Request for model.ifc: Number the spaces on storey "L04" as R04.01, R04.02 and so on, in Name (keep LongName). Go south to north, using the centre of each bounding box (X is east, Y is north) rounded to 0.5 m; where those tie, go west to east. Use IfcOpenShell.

First a look at what the model holds.

```python
import ifcopenshell
import ifcopenshell.util.element
import ifcopenshell.util.placement

model = ifcopenshell.open("model.ifc")
print(model.schema)
storey = next(s for s in model.by_type("IfcBuildingStorey") if s.Name == "L04")
spaces = [e for e in ifcopenshell.util.element.get_decomposition(storey) if e.is_a("IfcSpace")]
for e in sorted(spaces, key=lambda e: e.id()):
    origin = ifcopenshell.util.placement.get_local_placement(e.ObjectPlacement)[:3, 3]
    print(e.id(), e.Name, e.LongName, origin.round(2) + 0.0, sep=" | ")
```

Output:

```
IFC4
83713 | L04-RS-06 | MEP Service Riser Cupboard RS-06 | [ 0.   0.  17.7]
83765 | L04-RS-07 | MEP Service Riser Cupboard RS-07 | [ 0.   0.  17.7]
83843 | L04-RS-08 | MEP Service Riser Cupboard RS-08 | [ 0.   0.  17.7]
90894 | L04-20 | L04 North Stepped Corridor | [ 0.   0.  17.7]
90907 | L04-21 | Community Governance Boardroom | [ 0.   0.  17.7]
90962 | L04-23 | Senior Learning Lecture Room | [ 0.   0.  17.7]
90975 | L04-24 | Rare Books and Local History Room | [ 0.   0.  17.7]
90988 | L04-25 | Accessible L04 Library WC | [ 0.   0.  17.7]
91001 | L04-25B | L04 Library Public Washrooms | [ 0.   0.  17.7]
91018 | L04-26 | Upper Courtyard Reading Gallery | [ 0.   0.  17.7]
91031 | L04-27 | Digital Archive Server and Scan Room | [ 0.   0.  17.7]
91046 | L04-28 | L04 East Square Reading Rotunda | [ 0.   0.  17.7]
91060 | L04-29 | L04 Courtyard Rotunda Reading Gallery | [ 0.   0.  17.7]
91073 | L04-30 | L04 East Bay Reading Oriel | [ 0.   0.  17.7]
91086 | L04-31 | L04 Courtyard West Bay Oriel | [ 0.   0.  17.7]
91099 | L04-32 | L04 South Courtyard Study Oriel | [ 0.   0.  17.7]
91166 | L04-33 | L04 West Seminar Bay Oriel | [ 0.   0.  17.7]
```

```python
import ifcopenshell
import ifcopenshell.geom
import ifcopenshell.util.element
import ifcopenshell.util.shape

model = ifcopenshell.open("model.ifc")
settings = ifcopenshell.geom.settings()
settings.set("use-world-coords", True)


def centre(element):
    shape = ifcopenshell.geom.create_shape(settings, element)
    return ifcopenshell.util.shape.get_bbox_centroid(shape.geometry)


storey = next(s for s in model.by_type("IfcBuildingStorey") if s.Name == "L04")
spaces = [e for e in ifcopenshell.util.element.get_decomposition(storey) if e.is_a("IfcSpace")]

# Insertion points can sit at a corner or the storey origin, so sort by the geometry (in metres).
centres = {e: centre(e) for e in spaces}
spaces.sort(key=lambda e: (round(centres[e][1] / 0.5), centres[e][0]))

for i, e in enumerate(spaces, start=1):
    number = f"R04.{i:02d}"
    e.Name = number
    print(e.id(), number)

model.write("model_edited.ifc")
```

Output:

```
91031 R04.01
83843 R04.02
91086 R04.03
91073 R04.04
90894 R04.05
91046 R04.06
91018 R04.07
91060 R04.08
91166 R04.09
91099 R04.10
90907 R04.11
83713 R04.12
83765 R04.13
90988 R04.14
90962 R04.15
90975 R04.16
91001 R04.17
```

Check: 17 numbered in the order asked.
